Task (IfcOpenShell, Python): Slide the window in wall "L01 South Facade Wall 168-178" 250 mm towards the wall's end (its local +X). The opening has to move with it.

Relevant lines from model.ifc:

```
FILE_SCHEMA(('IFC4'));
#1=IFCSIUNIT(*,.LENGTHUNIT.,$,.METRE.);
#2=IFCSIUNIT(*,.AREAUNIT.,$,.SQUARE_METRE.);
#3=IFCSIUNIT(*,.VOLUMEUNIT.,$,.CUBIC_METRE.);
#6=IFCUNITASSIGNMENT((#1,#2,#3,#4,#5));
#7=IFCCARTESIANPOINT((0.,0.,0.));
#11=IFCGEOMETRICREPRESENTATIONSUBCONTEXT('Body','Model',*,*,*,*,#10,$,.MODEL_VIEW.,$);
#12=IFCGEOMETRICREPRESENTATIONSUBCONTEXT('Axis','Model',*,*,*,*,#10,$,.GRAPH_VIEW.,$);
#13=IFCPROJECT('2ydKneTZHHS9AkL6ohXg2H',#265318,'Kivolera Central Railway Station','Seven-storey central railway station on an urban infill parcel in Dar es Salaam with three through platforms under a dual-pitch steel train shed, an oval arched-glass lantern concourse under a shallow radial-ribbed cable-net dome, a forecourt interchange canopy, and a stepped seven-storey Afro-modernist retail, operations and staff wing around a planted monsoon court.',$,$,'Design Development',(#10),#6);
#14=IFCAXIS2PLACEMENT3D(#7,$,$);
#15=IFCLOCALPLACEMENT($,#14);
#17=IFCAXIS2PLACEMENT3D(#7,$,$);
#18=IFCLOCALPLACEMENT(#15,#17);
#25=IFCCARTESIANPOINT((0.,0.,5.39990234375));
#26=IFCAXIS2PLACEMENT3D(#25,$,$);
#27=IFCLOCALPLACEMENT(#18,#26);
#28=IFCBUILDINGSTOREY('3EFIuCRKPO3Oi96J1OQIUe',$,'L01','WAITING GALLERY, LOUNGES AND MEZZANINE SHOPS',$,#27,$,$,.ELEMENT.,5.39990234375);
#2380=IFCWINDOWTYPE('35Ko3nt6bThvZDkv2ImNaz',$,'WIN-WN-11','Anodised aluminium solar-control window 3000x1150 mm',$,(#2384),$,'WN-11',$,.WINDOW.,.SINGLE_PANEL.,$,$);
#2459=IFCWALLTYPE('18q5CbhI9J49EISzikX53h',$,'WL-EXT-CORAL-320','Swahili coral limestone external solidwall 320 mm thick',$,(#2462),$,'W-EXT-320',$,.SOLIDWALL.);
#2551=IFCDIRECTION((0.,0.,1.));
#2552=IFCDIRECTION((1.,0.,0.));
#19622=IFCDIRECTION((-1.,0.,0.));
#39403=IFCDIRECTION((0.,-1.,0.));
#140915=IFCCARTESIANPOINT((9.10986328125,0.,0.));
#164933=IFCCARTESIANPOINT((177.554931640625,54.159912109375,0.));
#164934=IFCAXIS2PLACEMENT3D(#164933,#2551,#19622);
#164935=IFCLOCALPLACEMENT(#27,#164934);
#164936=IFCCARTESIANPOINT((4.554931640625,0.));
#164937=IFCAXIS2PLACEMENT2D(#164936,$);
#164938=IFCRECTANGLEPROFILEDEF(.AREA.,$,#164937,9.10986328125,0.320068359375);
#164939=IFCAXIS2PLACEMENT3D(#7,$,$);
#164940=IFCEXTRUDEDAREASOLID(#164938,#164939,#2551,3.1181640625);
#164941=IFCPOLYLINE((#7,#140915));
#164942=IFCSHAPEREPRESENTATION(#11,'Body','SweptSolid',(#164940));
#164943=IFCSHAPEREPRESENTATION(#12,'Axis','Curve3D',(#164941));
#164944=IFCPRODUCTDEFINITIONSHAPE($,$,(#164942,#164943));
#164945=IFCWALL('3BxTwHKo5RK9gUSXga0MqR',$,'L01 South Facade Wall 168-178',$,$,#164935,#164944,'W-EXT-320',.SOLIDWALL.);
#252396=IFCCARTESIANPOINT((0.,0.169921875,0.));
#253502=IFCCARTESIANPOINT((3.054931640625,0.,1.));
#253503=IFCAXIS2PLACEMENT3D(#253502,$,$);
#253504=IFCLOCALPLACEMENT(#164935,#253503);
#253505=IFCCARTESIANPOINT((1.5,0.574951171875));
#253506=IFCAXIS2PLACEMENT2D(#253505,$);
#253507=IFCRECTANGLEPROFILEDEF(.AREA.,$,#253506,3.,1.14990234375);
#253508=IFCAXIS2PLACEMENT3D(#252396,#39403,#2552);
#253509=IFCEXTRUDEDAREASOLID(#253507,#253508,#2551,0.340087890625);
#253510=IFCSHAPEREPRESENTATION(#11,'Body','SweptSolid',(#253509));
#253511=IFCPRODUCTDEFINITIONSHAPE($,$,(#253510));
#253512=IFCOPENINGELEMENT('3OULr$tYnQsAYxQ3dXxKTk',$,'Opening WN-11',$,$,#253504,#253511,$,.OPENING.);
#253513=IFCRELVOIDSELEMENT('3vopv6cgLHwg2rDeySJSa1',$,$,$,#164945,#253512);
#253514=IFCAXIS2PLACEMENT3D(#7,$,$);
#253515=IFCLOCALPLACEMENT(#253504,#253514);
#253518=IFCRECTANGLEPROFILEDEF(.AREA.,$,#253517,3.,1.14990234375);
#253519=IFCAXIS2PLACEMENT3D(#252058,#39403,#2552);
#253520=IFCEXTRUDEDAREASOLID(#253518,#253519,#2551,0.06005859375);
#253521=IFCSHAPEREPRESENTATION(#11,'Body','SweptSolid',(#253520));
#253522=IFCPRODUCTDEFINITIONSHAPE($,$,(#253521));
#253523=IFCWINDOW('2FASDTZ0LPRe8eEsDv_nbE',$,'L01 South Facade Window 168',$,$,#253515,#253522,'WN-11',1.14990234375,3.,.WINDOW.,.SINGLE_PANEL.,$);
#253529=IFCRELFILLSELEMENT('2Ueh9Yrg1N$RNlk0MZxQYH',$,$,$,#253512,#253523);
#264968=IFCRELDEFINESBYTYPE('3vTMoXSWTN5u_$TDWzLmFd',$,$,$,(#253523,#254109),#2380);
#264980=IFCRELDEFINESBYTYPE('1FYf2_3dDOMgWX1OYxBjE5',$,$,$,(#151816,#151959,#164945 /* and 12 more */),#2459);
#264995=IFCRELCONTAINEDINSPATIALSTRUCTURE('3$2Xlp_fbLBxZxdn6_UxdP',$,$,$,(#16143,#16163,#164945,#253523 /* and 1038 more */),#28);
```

```python
import ifcopenshell
import ifcopenshell.api.geometry
import ifcopenshell.util.placement
import ifcopenshell.util.unit

model = ifcopenshell.open("model.ifc")
unit_scale = ifcopenshell.util.unit.calculate_unit_scale(model)

window = model.by_id(253523)
opening = window.FillsVoids[0].RelatingOpeningElement
wall = opening.VoidsElements[0].RelatingBuildingElement

wall_matrix = ifcopenshell.util.placement.get_local_placement(wall.ObjectPlacement)
shift = wall_matrix[:3, 0] * 0.25 / unit_scale
before = ifcopenshell.util.placement.get_local_placement(window.ObjectPlacement)[:3, 3].copy()

# The window is placed relative to its opening, so it follows when the opening moves.
matrix = ifcopenshell.util.placement.get_local_placement(opening.ObjectPlacement)
matrix[:3, 3] += shift
ifcopenshell.api.geometry.edit_object_placement(
    model, product=opening, matrix=matrix, is_si=False, should_transform_children=True
)

after = ifcopenshell.util.placement.get_local_placement(window.ObjectPlacement)[:3, 3]
print("window moved by", (after - before).round(3) + 0.0)

model.write("model_updated.ifc")
```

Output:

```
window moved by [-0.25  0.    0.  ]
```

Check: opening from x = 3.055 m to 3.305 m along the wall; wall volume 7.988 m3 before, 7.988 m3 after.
